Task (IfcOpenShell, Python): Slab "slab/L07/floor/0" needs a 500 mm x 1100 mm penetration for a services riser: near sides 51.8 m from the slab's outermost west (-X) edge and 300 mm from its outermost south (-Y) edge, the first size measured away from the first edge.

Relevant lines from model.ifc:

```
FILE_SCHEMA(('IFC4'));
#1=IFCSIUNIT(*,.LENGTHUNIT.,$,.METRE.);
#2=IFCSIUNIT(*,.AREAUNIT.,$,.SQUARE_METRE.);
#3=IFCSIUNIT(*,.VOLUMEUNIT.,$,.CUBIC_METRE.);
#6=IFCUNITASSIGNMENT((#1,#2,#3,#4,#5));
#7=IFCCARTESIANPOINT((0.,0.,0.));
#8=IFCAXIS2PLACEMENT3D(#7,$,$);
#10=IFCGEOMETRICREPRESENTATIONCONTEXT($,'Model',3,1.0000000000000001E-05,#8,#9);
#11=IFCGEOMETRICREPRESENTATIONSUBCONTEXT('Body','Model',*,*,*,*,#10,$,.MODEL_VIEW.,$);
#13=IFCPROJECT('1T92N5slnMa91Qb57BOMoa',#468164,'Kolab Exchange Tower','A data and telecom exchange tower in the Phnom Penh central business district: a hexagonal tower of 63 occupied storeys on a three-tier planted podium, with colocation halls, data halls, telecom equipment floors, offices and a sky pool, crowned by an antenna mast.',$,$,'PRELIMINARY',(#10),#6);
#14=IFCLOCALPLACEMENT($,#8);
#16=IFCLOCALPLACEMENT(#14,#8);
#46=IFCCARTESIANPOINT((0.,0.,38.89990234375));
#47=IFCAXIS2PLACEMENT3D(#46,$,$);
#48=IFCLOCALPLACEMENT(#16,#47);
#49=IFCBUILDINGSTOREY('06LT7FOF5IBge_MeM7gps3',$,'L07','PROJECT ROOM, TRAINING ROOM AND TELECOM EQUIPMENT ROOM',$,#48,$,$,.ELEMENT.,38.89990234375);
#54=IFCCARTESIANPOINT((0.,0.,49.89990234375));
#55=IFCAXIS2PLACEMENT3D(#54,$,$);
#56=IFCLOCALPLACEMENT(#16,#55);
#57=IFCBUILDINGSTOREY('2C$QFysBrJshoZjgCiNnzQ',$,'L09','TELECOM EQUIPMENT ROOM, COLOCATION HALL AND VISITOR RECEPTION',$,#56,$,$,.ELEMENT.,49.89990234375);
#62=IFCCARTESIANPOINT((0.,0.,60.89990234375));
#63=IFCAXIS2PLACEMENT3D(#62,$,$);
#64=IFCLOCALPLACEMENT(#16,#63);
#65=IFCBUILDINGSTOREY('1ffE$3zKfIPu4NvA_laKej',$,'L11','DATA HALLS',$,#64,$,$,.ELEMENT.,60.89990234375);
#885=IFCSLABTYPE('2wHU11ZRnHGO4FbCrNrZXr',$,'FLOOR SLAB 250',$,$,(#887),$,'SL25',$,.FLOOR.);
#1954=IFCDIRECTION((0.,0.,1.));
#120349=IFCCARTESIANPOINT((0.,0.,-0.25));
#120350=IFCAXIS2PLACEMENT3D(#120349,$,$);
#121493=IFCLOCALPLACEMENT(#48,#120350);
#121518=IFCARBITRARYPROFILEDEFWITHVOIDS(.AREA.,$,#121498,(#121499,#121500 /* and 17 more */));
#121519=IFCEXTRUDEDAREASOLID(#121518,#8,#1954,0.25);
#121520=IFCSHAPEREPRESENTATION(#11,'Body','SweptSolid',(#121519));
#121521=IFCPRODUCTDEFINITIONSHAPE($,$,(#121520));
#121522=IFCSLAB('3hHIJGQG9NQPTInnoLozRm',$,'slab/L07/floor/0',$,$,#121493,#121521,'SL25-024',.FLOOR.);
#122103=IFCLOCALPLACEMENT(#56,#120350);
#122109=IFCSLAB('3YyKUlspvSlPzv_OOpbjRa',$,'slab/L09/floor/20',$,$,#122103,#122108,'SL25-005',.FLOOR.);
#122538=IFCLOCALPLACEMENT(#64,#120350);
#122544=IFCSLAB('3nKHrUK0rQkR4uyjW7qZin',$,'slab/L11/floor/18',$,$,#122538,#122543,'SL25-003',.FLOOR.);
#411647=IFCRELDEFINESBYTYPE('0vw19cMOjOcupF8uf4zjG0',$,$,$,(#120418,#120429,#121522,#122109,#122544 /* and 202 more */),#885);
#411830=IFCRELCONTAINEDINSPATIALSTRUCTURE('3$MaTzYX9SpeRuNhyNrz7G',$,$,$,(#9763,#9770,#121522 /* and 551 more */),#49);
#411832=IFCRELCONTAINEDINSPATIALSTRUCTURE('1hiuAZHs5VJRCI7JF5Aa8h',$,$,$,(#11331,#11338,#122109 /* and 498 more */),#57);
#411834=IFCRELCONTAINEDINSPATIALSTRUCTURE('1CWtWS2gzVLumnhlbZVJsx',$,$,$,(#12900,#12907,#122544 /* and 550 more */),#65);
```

```python
import numpy as np
import ifcopenshell
import ifcopenshell.api.feature
import ifcopenshell.api.geometry
import ifcopenshell.api.root
import ifcopenshell.geom
import ifcopenshell.util.placement
import ifcopenshell.util.representation
import ifcopenshell.util.shape
import ifcopenshell.util.unit

model = ifcopenshell.open("model.ifc")
unit_scale = ifcopenshell.util.unit.calculate_unit_scale(model)
settings = ifcopenshell.geom.settings()


def volume(element):
    """Net volume in cubic metres, openings subtracted."""
    shape = ifcopenshell.geom.create_shape(settings, element)
    return ifcopenshell.util.shape.get_volume(shape.geometry)


slab = model.by_guid("3hHIJGQG9NQPTInnoLozRm")
before = volume(slab)

# Extent in the slab's own axes, in metres. The edges named are its -X and -Y sides.
slab_shape = ifcopenshell.geom.create_shape(settings, slab)
vertices = ifcopenshell.util.shape.get_vertices(slab_shape.geometry)
x_min, y_min, bottom = vertices.min(axis=0)
top = vertices[:, 2].max()

opening = ifcopenshell.api.root.create_entity(model, ifc_class="IfcOpeningElement", name="Services riser opening", predefined_type="OPENING")
context = ifcopenshell.util.representation.get_context(model, "Model", "Body", "MODEL_VIEW")
width, depth = 0.5, 1.1
outline = [(0.0, 0.0), (width, 0.0), (width, depth), (0.0, depth), (0.0, 0.0)]
# Overshoot both faces by 50 mm so the cut is clean.
shape = ifcopenshell.api.geometry.add_slab_representation(
    model, context=context, depth=top - bottom + 0.1, polyline=outline
)
ifcopenshell.api.geometry.assign_representation(model, product=opening, representation=shape)

matrix = ifcopenshell.util.placement.get_local_placement(slab.ObjectPlacement)
matrix[:, 3] = matrix @ np.append(np.array([x_min + 51.8, y_min + 0.3, bottom - 0.05]) / unit_scale, 1.0)
ifcopenshell.api.geometry.edit_object_placement(model, product=opening, matrix=matrix, is_si=False)
ifcopenshell.api.feature.add_feature(model, feature=opening, element=slab)

after = volume(slab)

print(f"slab volume {before:.3f} -> {after:.3f} m3")

model.write("model_updated.ifc")
```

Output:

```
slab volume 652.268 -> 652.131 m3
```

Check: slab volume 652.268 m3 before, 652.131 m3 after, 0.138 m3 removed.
